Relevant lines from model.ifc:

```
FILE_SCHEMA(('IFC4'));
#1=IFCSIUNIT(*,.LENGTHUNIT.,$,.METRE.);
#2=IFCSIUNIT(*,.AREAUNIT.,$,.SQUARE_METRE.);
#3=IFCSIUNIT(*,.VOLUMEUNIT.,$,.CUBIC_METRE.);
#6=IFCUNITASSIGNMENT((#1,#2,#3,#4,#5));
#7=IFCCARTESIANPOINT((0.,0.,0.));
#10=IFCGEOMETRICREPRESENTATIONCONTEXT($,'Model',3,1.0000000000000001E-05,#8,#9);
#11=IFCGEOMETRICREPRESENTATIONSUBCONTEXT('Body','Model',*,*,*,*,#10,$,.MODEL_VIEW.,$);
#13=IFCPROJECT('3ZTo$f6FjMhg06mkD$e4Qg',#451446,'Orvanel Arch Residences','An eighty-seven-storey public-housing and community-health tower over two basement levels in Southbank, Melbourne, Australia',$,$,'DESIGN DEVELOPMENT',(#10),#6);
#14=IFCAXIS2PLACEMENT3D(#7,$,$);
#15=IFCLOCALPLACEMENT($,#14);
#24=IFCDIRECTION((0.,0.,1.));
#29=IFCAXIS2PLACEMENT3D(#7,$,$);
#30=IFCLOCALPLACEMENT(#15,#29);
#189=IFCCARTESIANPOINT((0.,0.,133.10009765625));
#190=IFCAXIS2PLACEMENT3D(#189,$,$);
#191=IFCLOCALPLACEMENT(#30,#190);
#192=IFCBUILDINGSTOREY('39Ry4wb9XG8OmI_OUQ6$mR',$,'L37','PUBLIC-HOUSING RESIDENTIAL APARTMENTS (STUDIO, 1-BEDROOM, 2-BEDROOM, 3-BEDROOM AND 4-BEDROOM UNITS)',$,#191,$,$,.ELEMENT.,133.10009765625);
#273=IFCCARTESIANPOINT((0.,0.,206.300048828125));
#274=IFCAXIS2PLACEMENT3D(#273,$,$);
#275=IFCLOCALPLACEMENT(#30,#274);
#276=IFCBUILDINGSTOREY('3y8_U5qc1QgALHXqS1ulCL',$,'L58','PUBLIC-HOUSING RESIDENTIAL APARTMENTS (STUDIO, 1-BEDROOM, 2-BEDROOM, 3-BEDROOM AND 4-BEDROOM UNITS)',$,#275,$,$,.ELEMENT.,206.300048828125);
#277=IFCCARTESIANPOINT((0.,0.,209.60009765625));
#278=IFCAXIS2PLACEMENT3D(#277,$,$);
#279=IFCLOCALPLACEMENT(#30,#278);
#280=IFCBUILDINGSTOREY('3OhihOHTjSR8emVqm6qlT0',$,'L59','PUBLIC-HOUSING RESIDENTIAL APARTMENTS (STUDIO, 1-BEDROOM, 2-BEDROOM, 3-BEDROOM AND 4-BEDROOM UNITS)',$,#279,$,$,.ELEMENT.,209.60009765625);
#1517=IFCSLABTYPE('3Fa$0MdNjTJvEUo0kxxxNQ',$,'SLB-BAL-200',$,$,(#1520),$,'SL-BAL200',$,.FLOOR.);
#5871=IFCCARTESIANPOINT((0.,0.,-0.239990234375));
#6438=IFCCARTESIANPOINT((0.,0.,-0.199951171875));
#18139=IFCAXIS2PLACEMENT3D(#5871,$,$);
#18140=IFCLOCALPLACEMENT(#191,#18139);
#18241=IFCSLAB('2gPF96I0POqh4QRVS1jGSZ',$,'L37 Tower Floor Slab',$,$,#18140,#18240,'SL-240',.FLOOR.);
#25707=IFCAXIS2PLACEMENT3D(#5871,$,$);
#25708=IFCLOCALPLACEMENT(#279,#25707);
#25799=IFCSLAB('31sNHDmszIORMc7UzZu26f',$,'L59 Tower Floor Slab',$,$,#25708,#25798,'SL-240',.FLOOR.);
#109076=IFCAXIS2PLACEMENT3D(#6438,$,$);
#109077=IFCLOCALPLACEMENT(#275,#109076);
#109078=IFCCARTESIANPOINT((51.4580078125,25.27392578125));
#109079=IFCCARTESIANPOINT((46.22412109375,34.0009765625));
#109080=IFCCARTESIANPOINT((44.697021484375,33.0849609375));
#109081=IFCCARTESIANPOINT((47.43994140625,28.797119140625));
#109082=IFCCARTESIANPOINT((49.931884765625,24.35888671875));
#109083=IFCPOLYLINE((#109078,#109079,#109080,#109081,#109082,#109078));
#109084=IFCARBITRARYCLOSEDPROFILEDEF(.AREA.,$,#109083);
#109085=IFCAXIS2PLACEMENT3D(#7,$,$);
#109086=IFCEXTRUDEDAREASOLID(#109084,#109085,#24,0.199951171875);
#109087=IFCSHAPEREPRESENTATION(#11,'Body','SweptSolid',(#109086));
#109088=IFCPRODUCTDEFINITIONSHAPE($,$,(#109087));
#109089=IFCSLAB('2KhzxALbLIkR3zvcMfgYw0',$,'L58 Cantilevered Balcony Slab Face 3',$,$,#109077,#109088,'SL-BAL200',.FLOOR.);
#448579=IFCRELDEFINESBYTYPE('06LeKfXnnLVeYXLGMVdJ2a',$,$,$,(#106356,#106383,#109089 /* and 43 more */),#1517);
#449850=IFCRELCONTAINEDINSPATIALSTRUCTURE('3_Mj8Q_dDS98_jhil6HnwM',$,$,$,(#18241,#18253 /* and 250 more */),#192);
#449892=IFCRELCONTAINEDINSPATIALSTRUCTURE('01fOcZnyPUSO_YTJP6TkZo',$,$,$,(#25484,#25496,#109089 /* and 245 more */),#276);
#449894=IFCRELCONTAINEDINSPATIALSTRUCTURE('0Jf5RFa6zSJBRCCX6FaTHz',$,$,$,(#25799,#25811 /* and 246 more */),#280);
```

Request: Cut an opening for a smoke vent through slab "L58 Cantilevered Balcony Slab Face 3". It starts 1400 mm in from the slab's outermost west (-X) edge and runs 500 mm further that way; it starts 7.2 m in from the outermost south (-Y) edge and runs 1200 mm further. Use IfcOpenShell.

```python
import numpy as np
import ifcopenshell
import ifcopenshell.api.feature
import ifcopenshell.api.geometry
import ifcopenshell.api.root
import ifcopenshell.geom
import ifcopenshell.util.placement
import ifcopenshell.util.representation
import ifcopenshell.util.shape
import ifcopenshell.util.unit

model = ifcopenshell.open("model.ifc")
unit_scale = ifcopenshell.util.unit.calculate_unit_scale(model)
settings = ifcopenshell.geom.settings()


def volume(element):
    """Net volume in cubic metres, openings subtracted."""
    shape = ifcopenshell.geom.create_shape(settings, element)
    return ifcopenshell.util.shape.get_volume(shape.geometry)


slab = model.by_id(109089)
before = volume(slab)

# Extent in the slab's own axes, in metres. The edges named are its -X and -Y sides.
slab_shape = ifcopenshell.geom.create_shape(settings, slab)
vertices = ifcopenshell.util.shape.get_vertices(slab_shape.geometry)
x_min, y_min, bottom = vertices.min(axis=0)
top = vertices[:, 2].max()

opening = ifcopenshell.api.root.create_entity(model, ifc_class="IfcOpeningElement", name="Smoke vent opening", predefined_type="OPENING")
context = ifcopenshell.util.representation.get_context(model, "Model", "Body", "MODEL_VIEW")
width, depth = 0.5, 1.2
outline = [(0.0, 0.0), (width, 0.0), (width, depth), (0.0, depth), (0.0, 0.0)]
# Overshoot both faces by 50 mm so the cut is clean.
shape = ifcopenshell.api.geometry.add_slab_representation(
    model, context=context, depth=top - bottom + 0.1, polyline=outline
)
ifcopenshell.api.geometry.assign_representation(model, product=opening, representation=shape)

matrix = ifcopenshell.util.placement.get_local_placement(slab.ObjectPlacement)
matrix[:, 3] = matrix @ np.append(np.array([x_min + 1.4, y_min + 7.2, bottom - 0.05]) / unit_scale, 1.0)
ifcopenshell.api.geometry.edit_object_placement(model, product=opening, matrix=matrix, is_si=False)
ifcopenshell.api.feature.add_feature(model, feature=opening, element=slab)

after = volume(slab)

print(f"slab volume {before:.3f} -> {after:.3f} m3")

model.write("model_rev.ifc")
```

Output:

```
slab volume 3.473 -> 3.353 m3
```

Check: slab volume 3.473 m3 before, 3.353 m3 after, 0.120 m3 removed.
